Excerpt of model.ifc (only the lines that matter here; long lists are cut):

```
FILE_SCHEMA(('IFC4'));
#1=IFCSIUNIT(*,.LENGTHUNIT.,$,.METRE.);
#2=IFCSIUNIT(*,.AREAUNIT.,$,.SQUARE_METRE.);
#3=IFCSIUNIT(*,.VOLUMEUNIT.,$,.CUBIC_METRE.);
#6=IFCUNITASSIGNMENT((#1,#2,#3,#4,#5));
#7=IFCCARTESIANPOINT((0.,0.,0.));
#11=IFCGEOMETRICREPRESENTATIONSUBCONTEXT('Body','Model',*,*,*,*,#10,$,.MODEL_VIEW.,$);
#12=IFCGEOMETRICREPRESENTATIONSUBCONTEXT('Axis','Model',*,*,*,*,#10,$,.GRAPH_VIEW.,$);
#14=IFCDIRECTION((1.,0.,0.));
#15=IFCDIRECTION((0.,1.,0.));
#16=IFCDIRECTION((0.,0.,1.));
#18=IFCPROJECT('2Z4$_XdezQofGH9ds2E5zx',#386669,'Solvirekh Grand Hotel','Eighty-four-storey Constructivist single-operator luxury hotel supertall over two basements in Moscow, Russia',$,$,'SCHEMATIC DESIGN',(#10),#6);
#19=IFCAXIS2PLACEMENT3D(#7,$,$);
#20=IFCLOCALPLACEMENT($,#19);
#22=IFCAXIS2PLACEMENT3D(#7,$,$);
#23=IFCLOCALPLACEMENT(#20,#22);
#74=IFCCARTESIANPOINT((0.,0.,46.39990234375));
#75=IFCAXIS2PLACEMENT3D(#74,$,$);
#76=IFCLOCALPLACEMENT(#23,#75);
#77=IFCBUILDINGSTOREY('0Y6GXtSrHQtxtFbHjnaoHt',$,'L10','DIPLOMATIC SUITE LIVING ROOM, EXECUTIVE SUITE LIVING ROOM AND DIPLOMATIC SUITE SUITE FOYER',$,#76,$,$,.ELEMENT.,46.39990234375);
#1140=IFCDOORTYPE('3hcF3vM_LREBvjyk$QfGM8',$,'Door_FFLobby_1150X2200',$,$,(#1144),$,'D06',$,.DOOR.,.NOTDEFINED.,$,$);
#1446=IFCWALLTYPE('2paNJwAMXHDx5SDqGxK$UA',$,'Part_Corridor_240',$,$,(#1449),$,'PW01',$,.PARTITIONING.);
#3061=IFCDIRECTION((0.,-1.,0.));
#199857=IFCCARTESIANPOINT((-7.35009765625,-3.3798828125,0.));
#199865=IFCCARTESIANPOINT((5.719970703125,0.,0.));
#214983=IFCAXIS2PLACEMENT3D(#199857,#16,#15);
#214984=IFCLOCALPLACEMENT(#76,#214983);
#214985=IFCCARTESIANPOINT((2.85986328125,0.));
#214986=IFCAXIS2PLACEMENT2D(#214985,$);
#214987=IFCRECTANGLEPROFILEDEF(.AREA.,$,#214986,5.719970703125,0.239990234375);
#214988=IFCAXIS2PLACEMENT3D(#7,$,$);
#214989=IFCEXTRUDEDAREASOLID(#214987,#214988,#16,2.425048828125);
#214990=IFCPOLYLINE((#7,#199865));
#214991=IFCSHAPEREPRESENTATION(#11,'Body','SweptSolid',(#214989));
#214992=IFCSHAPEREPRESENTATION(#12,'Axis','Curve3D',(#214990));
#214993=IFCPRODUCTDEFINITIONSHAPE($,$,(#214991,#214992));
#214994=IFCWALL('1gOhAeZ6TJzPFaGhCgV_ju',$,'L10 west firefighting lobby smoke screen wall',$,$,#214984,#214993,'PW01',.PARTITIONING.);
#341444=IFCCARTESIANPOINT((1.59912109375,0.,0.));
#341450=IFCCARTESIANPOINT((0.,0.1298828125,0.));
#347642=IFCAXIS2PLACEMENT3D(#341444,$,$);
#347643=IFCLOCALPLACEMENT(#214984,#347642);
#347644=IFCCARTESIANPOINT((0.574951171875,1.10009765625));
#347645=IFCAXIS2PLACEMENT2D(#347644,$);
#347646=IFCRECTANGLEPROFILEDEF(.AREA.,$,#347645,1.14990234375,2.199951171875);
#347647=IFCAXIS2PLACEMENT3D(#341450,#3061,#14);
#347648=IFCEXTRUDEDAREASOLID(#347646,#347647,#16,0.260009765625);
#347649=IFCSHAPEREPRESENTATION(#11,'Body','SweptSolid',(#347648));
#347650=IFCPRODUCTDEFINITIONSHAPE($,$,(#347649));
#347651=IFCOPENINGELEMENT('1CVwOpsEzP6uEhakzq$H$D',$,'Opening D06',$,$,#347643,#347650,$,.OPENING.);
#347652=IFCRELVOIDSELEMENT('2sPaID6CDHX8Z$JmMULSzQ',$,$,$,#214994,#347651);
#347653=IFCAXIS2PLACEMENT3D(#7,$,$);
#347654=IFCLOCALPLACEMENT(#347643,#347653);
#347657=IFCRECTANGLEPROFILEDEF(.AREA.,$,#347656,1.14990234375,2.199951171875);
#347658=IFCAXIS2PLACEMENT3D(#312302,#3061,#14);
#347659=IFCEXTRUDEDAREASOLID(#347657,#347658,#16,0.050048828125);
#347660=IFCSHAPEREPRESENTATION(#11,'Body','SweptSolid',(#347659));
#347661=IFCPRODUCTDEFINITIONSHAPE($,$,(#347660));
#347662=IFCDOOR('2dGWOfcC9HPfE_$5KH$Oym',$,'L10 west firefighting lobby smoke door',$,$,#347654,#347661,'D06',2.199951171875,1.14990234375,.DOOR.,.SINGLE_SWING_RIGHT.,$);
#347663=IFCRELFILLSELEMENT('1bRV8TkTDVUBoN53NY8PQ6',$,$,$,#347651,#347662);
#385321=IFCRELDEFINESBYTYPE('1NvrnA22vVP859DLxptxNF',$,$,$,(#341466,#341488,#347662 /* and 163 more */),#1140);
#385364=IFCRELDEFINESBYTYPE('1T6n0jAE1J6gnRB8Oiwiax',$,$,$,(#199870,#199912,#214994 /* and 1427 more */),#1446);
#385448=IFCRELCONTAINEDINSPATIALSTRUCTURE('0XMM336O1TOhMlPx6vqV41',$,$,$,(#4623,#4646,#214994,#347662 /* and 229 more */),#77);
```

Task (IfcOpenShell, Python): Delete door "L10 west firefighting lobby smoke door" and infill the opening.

```python
import ifcopenshell
import ifcopenshell.api.feature
import ifcopenshell.api.root
import ifcopenshell.geom
import ifcopenshell.util.shape

model = ifcopenshell.open("model.ifc")
settings = ifcopenshell.geom.settings()


def volume(element):
    """Net volume in cubic metres, openings subtracted."""
    shape = ifcopenshell.geom.create_shape(settings, element)
    return ifcopenshell.util.shape.get_volume(shape.geometry)


door = model.by_guid("2dGWOfcC9HPfE_$5KH$Oym")
opening = door.FillsVoids[0].RelatingOpeningElement
wall = opening.VoidsElements[0].RelatingBuildingElement
before = volume(wall)

ifcopenshell.api.root.remove_product(model, product=door)
ifcopenshell.api.feature.remove_feature(model, feature=opening)

after = volume(wall)

print(f"wall volume {before:.3f} -> {after:.3f} m3")

model.write("model-out.ifc")
```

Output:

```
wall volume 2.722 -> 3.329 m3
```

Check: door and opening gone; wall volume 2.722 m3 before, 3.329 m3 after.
